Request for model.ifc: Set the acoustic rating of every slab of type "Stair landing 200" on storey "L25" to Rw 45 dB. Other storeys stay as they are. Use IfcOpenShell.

First a look at what the model holds.

```python
import ifcopenshell
import ifcopenshell.util.element

model = ifcopenshell.open("model.ifc")
print(model.schema)
storey = next(s for s in model.by_type("IfcBuildingStorey") if s.Name == "L25")
slabs = [e for e in ifcopenshell.util.element.get_decomposition(storey) if e.is_a("IfcSlab")]
seen = {}
for e in slabs:
    element_type = ifcopenshell.util.element.get_type(e)
    key = (element_type.Name if element_type != e and element_type else None, ifcopenshell.util.element.get_pset(e, "Pset_SlabCommon", "AcousticRating"))
    seen[key] = seen.get(key, 0) + 1
for (name, value), count in sorted(seen.items(), key=str):
    print(count, "x", name, "|", value)
```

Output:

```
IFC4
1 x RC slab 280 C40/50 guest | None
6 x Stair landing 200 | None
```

```python
import ifcopenshell
import ifcopenshell.api.pset
import ifcopenshell.util.element

model = ifcopenshell.open("model.ifc")

storey = next(s for s in model.by_type("IfcBuildingStorey") if s.Name == "L25")
slabs = [e for e in ifcopenshell.util.element.get_decomposition(storey) if e.is_a("IfcSlab")]

count = 0
for e in slabs:
    element_type = ifcopenshell.util.element.get_type(e)
    if element_type in (None, e) or element_type.Name != "Stair landing 200":
        continue
    # add_pset returns the element's existing set when there is one.
    pset = ifcopenshell.api.pset.add_pset(model, product=e, name="Pset_SlabCommon")
    ifcopenshell.api.pset.edit_pset(model, pset=pset, properties={"AcousticRating": "Rw 45 dB"})
    count += 1

print(count, "slabs updated")

model.write("model_edited.ifc")
```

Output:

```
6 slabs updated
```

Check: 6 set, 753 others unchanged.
